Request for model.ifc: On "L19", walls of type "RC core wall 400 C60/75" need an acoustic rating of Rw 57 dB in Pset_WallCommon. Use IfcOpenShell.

First a look at what the model holds.

```python
import ifcopenshell
import ifcopenshell.util.element

model = ifcopenshell.open("model.ifc")
print(model.schema)
storey = next(s for s in model.by_type("IfcBuildingStorey") if s.Name == "L19")
walls = [e for e in ifcopenshell.util.element.get_decomposition(storey) if e.is_a("IfcWall")]
seen = {}
for e in walls:
    element_type = ifcopenshell.util.element.get_type(e)
    key = (element_type.Name if element_type != e and element_type else None, ifcopenshell.util.element.get_pset(e, "Pset_WallCommon", "AcousticRating"))
    seen[key] = seen.get(key, 0) + 1
for (name, value), count in sorted(seen.items(), key=str):
    print(count, "x", name, "|", value)
```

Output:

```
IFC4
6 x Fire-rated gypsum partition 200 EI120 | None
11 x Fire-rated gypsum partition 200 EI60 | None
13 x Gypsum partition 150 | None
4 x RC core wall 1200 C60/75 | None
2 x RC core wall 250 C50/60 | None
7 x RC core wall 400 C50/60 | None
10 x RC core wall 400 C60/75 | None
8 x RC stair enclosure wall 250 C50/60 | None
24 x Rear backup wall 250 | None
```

```python
import ifcopenshell
import ifcopenshell.api.pset
import ifcopenshell.util.element

model = ifcopenshell.open("model.ifc")

storey = next(s for s in model.by_type("IfcBuildingStorey") if s.Name == "L19")
walls = [e for e in ifcopenshell.util.element.get_decomposition(storey) if e.is_a("IfcWall")]

count = 0
for e in walls:
    element_type = ifcopenshell.util.element.get_type(e)
    if element_type in (None, e) or element_type.Name != "RC core wall 400 C60/75":
        continue
    found = ifcopenshell.util.element.get_pset(e, "Pset_WallCommon", should_inherit=False)
    if found:
        pset = model.by_id(found["id"])
        if len(ifcopenshell.util.element.get_elements_by_pset(pset)) > 1:
            pset = ifcopenshell.api.pset.unshare_pset(model, products=[e], pset=pset)[0]
    else:
        pset = ifcopenshell.api.pset.add_pset(model, product=e, name="Pset_WallCommon")
    ifcopenshell.api.pset.edit_pset(model, pset=pset, properties={"AcousticRating": "Rw 57 dB"})
    count += 1

print(count, "walls updated")

model.write("model_edited.ifc")
```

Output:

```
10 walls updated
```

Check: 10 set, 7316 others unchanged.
